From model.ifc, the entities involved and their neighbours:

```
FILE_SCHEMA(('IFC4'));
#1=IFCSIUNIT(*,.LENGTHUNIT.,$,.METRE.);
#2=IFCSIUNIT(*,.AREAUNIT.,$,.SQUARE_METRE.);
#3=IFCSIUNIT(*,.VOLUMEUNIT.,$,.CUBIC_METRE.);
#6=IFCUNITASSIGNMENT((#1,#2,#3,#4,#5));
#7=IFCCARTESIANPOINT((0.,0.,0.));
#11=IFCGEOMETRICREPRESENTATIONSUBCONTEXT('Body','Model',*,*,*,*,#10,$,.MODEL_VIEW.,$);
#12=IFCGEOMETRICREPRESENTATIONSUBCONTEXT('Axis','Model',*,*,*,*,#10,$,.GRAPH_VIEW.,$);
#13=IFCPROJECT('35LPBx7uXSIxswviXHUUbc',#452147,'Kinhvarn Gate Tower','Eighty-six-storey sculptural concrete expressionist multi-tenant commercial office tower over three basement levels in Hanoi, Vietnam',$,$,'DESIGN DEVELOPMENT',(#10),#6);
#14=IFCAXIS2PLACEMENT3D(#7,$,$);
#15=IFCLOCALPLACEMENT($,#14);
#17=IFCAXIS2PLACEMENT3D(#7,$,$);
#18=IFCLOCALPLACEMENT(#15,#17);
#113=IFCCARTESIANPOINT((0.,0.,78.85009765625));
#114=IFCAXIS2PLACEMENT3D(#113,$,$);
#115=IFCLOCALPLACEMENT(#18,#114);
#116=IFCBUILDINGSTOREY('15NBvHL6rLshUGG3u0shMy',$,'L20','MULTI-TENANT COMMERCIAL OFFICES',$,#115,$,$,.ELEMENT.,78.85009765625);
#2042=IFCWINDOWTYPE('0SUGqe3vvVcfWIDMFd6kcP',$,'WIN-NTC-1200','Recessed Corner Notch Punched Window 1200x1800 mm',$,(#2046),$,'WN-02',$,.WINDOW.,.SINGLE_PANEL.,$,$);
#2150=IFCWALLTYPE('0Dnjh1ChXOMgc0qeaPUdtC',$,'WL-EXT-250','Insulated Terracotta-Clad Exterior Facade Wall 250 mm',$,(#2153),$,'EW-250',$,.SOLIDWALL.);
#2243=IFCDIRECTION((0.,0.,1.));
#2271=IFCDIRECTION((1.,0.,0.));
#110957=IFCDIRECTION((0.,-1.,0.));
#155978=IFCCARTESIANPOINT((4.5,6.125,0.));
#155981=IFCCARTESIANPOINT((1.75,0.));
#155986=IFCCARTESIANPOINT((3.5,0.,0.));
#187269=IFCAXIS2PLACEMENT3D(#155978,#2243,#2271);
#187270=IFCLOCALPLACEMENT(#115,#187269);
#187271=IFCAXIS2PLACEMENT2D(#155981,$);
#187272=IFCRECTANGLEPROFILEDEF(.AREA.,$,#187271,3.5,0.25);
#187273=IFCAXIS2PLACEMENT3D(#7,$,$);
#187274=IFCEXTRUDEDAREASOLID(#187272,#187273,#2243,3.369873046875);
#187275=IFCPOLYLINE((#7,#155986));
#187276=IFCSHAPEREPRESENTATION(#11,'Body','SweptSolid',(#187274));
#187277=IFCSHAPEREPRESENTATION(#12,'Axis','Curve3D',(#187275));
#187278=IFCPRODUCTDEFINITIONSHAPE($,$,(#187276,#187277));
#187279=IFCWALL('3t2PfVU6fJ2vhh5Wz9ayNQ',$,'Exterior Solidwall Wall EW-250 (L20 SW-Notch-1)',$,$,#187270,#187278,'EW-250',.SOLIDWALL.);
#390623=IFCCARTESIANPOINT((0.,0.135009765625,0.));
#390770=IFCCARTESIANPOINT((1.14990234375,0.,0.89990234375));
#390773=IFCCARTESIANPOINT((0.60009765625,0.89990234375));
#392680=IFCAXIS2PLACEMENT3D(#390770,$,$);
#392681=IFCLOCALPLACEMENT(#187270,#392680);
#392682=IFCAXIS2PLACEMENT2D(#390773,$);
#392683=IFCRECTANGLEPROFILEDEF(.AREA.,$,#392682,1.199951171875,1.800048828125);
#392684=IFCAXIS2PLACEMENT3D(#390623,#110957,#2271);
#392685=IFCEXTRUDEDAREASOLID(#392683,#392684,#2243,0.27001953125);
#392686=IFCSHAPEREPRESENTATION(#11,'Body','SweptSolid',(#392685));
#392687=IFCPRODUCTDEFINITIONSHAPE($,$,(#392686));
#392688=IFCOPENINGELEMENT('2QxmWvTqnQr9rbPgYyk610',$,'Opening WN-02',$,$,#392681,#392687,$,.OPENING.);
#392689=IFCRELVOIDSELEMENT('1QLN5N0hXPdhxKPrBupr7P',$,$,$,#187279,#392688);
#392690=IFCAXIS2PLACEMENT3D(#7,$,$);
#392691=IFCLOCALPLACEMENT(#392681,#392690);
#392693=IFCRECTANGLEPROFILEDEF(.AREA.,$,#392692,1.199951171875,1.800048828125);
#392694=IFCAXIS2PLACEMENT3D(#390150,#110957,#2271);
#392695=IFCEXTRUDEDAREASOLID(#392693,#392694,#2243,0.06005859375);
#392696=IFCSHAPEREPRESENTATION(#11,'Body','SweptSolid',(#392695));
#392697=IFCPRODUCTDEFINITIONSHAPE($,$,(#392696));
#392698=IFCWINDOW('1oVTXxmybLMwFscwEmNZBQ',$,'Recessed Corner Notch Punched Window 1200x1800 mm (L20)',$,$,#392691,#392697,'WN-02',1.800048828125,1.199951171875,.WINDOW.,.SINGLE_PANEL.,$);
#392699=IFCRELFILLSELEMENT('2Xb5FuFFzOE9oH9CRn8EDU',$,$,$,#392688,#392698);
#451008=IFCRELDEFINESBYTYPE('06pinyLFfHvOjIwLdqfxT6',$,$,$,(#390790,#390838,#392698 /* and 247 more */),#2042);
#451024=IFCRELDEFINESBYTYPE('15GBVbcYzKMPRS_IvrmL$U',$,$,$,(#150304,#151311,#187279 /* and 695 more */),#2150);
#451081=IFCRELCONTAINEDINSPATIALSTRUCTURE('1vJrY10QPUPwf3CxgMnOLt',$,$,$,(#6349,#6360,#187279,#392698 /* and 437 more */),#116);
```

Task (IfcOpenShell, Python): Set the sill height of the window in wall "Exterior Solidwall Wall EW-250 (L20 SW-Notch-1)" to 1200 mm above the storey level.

```python
import numpy as np
import ifcopenshell
import ifcopenshell.api.geometry
import ifcopenshell.geom
import ifcopenshell.util.element
import ifcopenshell.util.placement
import ifcopenshell.util.shape
import ifcopenshell.util.unit

model = ifcopenshell.open("model.ifc")
unit_scale = ifcopenshell.util.unit.calculate_unit_scale(model)

window = model.by_id(392698)
opening = window.FillsVoids[0].RelatingOpeningElement
storey = ifcopenshell.util.element.get_container(window, ifc_class="IfcBuildingStorey")
level = ifcopenshell.util.placement.get_local_placement(storey.ObjectPlacement)[2, 3]

# The opening's origin need not be at the sill, so measure its lowest point.
shape = ifcopenshell.geom.create_shape(ifcopenshell.geom.settings(), opening)
bottom = ifcopenshell.util.shape.get_shape_bottom_elevation(shape, shape.geometry) / unit_scale
dz = level + 1.2 - bottom

shift = np.array([0.0, 0.0, dz])
# The window is placed relative to its opening, so it follows when the opening moves.
matrix = ifcopenshell.util.placement.get_local_placement(opening.ObjectPlacement)
matrix[:3, 3] += shift
ifcopenshell.api.geometry.edit_object_placement(
    model, product=opening, matrix=matrix, is_si=False, should_transform_children=True
)

print(f"moved by {dz * unit_scale:+.3f} m")

model.write("model_updated.ifc")
```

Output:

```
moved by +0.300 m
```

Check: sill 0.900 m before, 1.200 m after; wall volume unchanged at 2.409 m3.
